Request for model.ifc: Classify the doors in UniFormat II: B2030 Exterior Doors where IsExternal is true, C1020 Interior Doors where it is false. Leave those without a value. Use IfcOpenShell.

First a look at what the model holds.

```python
import ifcopenshell
import ifcopenshell.util.element

model = ifcopenshell.open("model.ifc")
print(model.schema)
print("classifications:", [c.Name for c in model.by_type("IfcClassification")])
values = [ifcopenshell.util.element.get_pset(e, "Pset_DoorCommon", "IsExternal") for e in model.by_type("IfcDoor")]
for value in (True, False, None):
    print("IsExternal", value, values.count(value))
```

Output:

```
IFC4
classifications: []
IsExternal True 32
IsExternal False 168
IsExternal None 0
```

```python
import ifcopenshell
import ifcopenshell.api.classification
import ifcopenshell.util.element

model = ifcopenshell.open("model.ifc")

system = ifcopenshell.api.classification.add_classification(model, classification="UniFormat II")

doors = model.by_type("IfcDoor")
external = {e: ifcopenshell.util.element.get_pset(e, "Pset_DoorCommon", "IsExternal") for e in doors}
for flag, code, name in ((True, "B2030", "Exterior Doors"), (False, "C1020", "Interior Doors")):
    products = [e for e in doors if external[e] is flag]
    ifcopenshell.api.classification.add_reference(
        model, products=products, classification=system, identification=code, name=name
    )
    print(code, len(products))

model.write("model_updated.ifc")
```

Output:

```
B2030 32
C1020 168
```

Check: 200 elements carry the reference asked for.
